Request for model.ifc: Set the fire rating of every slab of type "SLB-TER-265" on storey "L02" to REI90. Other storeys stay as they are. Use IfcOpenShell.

First a look at what the model holds.

```python
import ifcopenshell
import ifcopenshell.util.element

model = ifcopenshell.open("model.ifc")
print(model.schema)
storey = next(s for s in model.by_type("IfcBuildingStorey") if s.Name == "L02")
slabs = [e for e in ifcopenshell.util.element.get_decomposition(storey) if e.is_a("IfcSlab")]
seen = {}
for e in slabs:
    element_type = ifcopenshell.util.element.get_type(e)
    key = (element_type.Name if element_type != e and element_type else None, ifcopenshell.util.element.get_pset(e, "Pset_SlabCommon", "FireRating"))
    seen[key] = seen.get(key, 0) + 1
for (name, value), count in sorted(seen.items(), key=str):
    print(count, "x", name, "|", value)
```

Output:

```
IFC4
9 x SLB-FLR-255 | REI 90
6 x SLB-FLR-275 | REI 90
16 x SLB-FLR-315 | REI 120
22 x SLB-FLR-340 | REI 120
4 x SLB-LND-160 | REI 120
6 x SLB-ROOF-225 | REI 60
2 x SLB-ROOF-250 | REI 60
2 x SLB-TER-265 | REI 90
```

```python
import ifcopenshell
import ifcopenshell.api.pset
import ifcopenshell.util.element

model = ifcopenshell.open("model.ifc")

storey = next(s for s in model.by_type("IfcBuildingStorey") if s.Name == "L02")
slabs = [e for e in ifcopenshell.util.element.get_decomposition(storey) if e.is_a("IfcSlab")]

count = 0
for e in slabs:
    element_type = ifcopenshell.util.element.get_type(e)
    if element_type in (None, e) or element_type.Name != "SLB-TER-265":
        continue
    # add_pset returns the element's existing set when there is one.
    pset = ifcopenshell.api.pset.add_pset(model, product=e, name="Pset_SlabCommon")
    ifcopenshell.api.pset.edit_pset(model, pset=pset, properties={"FireRating": "REI90"})
    count += 1

print(count, "slabs updated")

model.write("model_v2.ifc")
```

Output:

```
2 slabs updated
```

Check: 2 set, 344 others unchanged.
